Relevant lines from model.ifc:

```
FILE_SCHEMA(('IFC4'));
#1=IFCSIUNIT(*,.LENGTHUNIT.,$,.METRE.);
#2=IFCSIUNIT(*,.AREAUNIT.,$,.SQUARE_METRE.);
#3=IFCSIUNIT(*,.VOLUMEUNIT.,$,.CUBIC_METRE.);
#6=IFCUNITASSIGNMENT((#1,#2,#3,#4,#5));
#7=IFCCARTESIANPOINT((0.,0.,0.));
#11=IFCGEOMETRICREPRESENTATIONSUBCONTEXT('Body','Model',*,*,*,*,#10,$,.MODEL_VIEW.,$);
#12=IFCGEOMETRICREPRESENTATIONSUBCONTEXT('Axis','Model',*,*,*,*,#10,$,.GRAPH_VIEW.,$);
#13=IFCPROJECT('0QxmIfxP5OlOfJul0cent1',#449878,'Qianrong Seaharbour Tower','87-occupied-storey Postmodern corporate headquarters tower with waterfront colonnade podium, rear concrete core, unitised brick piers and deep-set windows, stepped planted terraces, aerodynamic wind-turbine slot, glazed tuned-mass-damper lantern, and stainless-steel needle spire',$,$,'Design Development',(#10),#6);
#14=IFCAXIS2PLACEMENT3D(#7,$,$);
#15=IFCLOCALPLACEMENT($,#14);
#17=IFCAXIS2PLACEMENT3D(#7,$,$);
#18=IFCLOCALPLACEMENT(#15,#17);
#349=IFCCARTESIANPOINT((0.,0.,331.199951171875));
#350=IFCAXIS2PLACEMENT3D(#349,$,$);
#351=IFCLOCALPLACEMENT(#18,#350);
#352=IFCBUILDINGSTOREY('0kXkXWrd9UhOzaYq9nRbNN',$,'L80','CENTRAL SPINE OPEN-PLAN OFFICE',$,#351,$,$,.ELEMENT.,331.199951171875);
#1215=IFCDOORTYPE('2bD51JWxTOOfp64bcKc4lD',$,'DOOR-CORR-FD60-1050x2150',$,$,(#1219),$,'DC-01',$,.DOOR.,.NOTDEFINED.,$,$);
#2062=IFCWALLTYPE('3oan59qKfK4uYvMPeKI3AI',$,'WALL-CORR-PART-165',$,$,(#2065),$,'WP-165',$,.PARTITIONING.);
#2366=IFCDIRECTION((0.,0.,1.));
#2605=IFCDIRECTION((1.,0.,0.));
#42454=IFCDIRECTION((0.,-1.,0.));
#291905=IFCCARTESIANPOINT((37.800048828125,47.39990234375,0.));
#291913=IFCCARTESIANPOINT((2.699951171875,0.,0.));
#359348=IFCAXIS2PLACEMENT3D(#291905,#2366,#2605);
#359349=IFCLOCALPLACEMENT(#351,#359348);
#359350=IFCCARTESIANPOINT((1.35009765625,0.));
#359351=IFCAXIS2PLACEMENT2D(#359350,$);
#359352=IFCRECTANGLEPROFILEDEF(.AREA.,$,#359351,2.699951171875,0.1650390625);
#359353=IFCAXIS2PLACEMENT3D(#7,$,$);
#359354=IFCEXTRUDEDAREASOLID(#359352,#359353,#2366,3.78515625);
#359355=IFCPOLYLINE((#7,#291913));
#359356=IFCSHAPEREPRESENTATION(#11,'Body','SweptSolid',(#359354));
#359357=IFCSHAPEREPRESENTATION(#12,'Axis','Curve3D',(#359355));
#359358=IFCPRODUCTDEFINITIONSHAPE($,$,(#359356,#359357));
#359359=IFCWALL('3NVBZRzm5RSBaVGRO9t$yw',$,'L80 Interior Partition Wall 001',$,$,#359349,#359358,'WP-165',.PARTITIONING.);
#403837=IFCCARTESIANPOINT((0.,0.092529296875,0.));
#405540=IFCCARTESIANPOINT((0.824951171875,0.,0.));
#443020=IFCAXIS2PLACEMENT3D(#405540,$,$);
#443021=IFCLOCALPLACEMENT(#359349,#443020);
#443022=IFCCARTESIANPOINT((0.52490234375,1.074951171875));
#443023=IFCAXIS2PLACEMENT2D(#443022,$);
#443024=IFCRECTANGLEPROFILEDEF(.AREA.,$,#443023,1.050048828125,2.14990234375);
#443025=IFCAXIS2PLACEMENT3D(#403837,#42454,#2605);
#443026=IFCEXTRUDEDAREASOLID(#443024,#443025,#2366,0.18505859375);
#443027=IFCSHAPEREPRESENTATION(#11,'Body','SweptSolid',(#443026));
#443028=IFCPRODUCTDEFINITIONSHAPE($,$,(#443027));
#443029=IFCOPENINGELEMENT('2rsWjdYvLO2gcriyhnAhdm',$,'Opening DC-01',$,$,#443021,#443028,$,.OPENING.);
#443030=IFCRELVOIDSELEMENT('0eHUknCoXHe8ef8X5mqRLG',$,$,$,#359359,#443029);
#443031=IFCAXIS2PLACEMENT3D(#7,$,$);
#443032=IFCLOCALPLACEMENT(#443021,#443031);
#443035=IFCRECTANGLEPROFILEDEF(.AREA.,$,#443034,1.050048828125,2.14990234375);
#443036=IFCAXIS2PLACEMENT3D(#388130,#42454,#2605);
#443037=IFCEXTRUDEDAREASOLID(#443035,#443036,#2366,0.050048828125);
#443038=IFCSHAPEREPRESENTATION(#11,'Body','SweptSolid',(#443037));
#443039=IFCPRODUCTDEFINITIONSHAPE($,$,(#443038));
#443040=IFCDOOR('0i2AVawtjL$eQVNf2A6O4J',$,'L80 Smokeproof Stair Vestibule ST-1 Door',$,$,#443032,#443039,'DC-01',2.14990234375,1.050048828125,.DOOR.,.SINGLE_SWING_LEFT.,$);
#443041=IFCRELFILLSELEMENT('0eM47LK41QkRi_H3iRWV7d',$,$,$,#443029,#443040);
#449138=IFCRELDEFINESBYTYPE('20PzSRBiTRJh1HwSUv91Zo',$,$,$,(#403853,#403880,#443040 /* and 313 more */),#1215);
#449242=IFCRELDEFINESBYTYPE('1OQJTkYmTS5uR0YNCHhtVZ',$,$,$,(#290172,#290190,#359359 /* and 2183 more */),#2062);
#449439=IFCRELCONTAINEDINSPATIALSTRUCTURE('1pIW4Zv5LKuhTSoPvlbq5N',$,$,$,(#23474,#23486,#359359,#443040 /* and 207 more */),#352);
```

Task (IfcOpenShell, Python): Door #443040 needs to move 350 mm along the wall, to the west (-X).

```python
import ifcopenshell
import ifcopenshell.api.geometry
import ifcopenshell.util.placement
import ifcopenshell.util.unit

model = ifcopenshell.open("model.ifc")
unit_scale = ifcopenshell.util.unit.calculate_unit_scale(model)

door = model.by_id(443040)
opening = door.FillsVoids[0].RelatingOpeningElement
wall = opening.VoidsElements[0].RelatingBuildingElement

wall_matrix = ifcopenshell.util.placement.get_local_placement(wall.ObjectPlacement)
shift = wall_matrix[:3, 0] * -0.35 / unit_scale
before = ifcopenshell.util.placement.get_local_placement(door.ObjectPlacement)[:3, 3].copy()

# The door is placed relative to its opening, so it follows when the opening moves.
matrix = ifcopenshell.util.placement.get_local_placement(opening.ObjectPlacement)
matrix[:3, 3] += shift
ifcopenshell.api.geometry.edit_object_placement(
    model, product=opening, matrix=matrix, is_si=False, should_transform_children=True
)

after = ifcopenshell.util.placement.get_local_placement(door.ObjectPlacement)[:3, 3]
print("door moved by", (after - before).round(3) + 0.0)

model.write("model-out.ifc")
```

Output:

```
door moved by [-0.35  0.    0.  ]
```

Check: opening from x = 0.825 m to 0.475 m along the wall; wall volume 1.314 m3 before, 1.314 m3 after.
